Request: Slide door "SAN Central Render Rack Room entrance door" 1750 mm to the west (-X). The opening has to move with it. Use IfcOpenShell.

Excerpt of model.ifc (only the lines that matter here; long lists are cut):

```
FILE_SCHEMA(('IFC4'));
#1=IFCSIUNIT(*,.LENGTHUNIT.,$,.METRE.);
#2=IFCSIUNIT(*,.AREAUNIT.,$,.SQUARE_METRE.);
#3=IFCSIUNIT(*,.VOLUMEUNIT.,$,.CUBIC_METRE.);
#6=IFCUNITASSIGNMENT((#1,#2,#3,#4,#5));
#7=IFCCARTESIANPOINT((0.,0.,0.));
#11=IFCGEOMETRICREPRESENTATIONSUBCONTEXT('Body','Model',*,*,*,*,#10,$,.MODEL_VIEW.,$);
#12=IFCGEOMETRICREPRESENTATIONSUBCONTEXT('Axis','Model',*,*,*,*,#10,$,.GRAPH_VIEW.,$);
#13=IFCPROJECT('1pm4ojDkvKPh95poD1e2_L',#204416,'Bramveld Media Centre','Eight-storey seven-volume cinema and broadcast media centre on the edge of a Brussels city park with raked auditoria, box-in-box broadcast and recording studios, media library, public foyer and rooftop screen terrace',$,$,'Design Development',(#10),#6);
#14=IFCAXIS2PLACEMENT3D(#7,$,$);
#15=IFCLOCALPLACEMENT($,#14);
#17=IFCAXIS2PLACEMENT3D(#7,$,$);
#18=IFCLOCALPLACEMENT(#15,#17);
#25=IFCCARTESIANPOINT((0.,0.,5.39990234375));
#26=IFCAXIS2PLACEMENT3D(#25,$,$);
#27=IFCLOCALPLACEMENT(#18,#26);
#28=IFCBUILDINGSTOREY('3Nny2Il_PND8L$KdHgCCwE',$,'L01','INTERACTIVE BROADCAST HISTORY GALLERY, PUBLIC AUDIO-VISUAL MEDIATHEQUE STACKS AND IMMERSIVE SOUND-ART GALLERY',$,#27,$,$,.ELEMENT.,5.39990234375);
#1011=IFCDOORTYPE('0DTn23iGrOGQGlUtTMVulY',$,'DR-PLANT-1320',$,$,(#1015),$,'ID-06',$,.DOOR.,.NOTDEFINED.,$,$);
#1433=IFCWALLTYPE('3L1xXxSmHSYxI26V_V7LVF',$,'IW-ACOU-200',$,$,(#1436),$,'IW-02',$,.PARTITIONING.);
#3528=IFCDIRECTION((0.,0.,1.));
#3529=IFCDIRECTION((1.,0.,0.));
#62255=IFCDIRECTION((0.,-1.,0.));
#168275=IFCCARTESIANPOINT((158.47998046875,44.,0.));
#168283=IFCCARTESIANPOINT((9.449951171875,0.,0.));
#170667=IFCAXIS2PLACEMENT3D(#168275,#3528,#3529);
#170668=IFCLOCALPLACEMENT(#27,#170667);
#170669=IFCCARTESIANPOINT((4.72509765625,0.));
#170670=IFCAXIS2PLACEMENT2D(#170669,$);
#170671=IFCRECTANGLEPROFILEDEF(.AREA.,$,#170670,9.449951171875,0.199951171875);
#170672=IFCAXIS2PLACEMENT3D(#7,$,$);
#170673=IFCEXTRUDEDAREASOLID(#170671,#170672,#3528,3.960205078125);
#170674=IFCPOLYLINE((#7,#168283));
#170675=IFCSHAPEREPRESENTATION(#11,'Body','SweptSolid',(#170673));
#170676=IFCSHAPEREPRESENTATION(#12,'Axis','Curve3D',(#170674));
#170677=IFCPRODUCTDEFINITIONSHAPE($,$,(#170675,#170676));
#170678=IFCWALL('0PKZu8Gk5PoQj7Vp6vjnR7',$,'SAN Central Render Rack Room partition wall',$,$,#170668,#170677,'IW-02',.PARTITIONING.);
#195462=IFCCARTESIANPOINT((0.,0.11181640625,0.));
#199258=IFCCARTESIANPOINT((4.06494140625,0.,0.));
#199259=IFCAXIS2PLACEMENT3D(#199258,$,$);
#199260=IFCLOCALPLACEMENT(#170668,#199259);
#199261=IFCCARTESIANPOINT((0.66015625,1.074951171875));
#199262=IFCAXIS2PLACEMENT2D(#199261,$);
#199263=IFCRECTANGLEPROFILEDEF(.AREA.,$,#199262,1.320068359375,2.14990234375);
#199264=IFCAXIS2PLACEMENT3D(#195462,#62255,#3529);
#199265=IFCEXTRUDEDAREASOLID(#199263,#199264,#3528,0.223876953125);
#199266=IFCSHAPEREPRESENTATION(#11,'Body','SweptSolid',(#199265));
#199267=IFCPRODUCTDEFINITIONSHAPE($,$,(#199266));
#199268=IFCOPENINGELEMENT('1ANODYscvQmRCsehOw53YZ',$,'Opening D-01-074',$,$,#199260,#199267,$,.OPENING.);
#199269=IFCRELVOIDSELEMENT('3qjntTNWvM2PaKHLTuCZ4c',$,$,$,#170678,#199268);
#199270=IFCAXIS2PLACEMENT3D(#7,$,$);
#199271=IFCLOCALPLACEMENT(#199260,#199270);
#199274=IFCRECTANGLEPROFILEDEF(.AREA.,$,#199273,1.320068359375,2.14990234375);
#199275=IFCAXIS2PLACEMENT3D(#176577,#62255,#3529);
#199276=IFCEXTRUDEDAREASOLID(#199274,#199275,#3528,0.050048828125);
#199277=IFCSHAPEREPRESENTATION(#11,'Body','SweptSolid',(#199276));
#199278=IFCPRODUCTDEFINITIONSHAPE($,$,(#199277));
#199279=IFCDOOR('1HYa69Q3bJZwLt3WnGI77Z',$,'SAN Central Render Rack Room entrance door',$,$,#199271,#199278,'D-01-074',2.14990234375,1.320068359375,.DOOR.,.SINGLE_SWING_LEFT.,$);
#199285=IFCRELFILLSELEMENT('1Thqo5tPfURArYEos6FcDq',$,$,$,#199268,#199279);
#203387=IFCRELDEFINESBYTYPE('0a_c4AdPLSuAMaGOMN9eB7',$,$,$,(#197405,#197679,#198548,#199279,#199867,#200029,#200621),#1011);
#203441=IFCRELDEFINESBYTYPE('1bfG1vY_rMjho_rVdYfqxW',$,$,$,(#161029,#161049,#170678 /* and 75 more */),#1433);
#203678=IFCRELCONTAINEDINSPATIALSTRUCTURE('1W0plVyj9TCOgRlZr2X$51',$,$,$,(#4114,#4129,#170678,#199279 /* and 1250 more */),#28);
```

```python
import ifcopenshell
import ifcopenshell.api.geometry
import ifcopenshell.util.placement
import ifcopenshell.util.unit

model = ifcopenshell.open("model.ifc")
unit_scale = ifcopenshell.util.unit.calculate_unit_scale(model)

door = model.by_guid("1HYa69Q3bJZwLt3WnGI77Z")
opening = door.FillsVoids[0].RelatingOpeningElement
wall = opening.VoidsElements[0].RelatingBuildingElement

wall_matrix = ifcopenshell.util.placement.get_local_placement(wall.ObjectPlacement)
shift = wall_matrix[:3, 0] * -1.75 / unit_scale
before = ifcopenshell.util.placement.get_local_placement(door.ObjectPlacement)[:3, 3].copy()

# The door is placed relative to its opening, so it follows when the opening moves.
matrix = ifcopenshell.util.placement.get_local_placement(opening.ObjectPlacement)
matrix[:3, 3] += shift
ifcopenshell.api.geometry.edit_object_placement(
    model, product=opening, matrix=matrix, is_si=False, should_transform_children=True
)

after = ifcopenshell.util.placement.get_local_placement(door.ObjectPlacement)[:3, 3]
print("door moved by", (after - before).round(3) + 0.0)

model.write("model_v2.ifc")
```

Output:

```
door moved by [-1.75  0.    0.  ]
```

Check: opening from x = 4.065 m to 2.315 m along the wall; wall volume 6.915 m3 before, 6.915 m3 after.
